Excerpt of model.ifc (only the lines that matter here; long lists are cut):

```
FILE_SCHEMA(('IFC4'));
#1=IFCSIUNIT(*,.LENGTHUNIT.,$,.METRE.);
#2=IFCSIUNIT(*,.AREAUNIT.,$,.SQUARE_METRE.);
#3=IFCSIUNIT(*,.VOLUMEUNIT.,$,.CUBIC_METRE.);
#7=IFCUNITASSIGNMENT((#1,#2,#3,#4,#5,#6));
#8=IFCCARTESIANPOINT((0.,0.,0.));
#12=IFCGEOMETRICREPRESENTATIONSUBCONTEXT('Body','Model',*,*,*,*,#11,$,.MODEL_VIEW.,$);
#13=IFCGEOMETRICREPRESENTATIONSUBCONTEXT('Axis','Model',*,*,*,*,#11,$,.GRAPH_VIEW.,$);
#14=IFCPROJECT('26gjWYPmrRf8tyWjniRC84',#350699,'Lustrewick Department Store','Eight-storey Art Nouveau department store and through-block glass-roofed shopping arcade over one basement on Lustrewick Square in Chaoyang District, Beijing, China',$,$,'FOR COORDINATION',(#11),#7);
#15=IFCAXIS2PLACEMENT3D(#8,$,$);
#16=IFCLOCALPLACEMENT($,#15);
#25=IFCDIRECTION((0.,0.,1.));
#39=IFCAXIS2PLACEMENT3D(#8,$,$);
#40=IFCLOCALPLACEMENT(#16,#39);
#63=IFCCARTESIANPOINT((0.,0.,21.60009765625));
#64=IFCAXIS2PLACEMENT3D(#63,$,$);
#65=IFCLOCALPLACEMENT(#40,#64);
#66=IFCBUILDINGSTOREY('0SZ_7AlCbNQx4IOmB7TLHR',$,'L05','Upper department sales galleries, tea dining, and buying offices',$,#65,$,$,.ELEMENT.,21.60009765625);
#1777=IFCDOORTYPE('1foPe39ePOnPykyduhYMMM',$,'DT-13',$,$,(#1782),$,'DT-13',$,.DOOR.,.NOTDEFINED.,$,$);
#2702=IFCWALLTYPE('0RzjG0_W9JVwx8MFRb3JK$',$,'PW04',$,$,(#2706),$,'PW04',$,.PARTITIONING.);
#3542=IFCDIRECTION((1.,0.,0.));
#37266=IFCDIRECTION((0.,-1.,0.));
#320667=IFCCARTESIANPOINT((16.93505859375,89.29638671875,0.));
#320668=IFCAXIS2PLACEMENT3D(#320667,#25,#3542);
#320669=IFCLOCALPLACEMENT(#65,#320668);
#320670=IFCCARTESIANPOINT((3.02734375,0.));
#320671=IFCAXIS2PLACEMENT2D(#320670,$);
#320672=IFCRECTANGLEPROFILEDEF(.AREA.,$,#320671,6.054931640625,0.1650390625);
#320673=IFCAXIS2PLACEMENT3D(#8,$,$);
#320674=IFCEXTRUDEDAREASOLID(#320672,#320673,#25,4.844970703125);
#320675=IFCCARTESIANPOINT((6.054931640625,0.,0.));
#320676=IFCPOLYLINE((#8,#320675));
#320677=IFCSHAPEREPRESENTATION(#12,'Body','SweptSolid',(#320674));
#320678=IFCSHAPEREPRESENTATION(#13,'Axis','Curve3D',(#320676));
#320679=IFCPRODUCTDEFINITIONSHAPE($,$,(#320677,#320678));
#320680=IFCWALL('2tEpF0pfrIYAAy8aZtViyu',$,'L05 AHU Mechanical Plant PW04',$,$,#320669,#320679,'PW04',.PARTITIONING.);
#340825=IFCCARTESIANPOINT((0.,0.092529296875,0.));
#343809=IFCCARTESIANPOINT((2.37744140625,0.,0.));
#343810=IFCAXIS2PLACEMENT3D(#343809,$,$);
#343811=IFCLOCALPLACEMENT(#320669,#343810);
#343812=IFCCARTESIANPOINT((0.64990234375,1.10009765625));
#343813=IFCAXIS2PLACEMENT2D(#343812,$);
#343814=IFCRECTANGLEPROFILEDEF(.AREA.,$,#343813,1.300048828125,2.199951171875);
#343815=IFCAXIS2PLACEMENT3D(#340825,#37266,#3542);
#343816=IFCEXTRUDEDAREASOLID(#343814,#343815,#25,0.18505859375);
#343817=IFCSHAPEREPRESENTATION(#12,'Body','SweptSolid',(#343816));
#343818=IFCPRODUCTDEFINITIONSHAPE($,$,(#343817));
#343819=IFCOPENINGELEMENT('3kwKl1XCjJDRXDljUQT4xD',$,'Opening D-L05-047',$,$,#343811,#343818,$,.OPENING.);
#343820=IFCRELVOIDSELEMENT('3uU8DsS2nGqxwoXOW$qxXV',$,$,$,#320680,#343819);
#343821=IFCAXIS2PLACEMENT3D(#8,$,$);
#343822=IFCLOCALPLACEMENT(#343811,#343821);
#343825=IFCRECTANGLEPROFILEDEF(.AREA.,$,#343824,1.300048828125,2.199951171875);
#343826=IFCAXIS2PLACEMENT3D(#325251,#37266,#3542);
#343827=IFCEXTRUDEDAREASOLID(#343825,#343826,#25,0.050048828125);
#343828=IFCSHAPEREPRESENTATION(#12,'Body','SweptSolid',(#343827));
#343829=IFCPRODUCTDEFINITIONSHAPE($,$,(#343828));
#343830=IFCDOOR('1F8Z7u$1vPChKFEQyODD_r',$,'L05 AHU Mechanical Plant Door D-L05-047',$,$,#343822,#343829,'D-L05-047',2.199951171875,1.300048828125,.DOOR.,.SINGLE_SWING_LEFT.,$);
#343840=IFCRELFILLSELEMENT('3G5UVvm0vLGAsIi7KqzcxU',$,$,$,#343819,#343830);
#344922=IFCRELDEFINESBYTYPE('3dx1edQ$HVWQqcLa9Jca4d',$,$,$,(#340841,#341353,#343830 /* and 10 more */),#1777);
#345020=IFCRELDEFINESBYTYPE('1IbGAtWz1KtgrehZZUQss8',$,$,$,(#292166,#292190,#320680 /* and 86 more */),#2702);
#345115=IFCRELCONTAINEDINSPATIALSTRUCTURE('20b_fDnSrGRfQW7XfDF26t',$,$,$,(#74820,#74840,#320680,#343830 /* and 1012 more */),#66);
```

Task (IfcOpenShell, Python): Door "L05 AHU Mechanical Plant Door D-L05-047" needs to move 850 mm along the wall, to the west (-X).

```python
import ifcopenshell
import ifcopenshell.api.geometry
import ifcopenshell.util.placement

model = ifcopenshell.open("model.ifc")

door = model.by_guid("1F8Z7u$1vPChKFEQyODD_r")
opening = door.FillsVoids[0].RelatingOpeningElement
wall = opening.VoidsElements[0].RelatingBuildingElement

wall_matrix = ifcopenshell.util.placement.get_local_placement(wall.ObjectPlacement)
shift = wall_matrix[:3, 0] * -0.85
before = ifcopenshell.util.placement.get_local_placement(door.ObjectPlacement)[:3, 3].copy()

# The door is placed relative to its opening, so it follows when the opening moves.
matrix = ifcopenshell.util.placement.get_local_placement(opening.ObjectPlacement)
matrix[:3, 3] += shift
ifcopenshell.api.geometry.edit_object_placement(
    model, product=opening, matrix=matrix, is_si=False, should_transform_children=True
)

after = ifcopenshell.util.placement.get_local_placement(door.ObjectPlacement)[:3, 3]
print("door moved by", (after - before).round(3) + 0.0)

model.write("model_rev.ifc")
```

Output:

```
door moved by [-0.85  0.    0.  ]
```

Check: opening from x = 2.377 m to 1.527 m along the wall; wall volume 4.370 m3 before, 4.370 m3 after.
